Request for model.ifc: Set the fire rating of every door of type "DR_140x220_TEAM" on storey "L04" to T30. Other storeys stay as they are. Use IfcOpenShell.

First a look at what the model holds.

```python
import ifcopenshell
import ifcopenshell.util.element

model = ifcopenshell.open("model.ifc")
print(model.schema)
storey = next(s for s in model.by_type("IfcBuildingStorey") if s.Name == "L04")
doors = [e for e in ifcopenshell.util.element.get_decomposition(storey) if e.is_a("IfcDoor")]
seen = {}
for e in doors:
    element_type = ifcopenshell.util.element.get_type(e)
    key = (element_type.Name if element_type != e and element_type else None, ifcopenshell.util.element.get_pset(e, "Pset_DoorCommon", "FireRating"))
    seen[key] = seen.get(key, 0) + 1
for (name, value), count in sorted(seen.items(), key=str):
    print(count, "x", name, "|", value)
```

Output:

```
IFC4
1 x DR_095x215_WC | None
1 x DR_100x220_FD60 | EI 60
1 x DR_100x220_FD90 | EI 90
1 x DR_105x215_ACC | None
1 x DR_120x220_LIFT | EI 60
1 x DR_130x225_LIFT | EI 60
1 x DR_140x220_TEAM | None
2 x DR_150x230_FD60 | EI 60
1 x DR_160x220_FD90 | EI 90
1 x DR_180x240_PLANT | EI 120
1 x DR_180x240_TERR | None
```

```python
import ifcopenshell
import ifcopenshell.api.pset
import ifcopenshell.util.element

model = ifcopenshell.open("model.ifc")

storey = next(s for s in model.by_type("IfcBuildingStorey") if s.Name == "L04")
doors = [e for e in ifcopenshell.util.element.get_decomposition(storey) if e.is_a("IfcDoor")]

count = 0
for e in doors:
    element_type = ifcopenshell.util.element.get_type(e)
    if element_type in (None, e) or element_type.Name != "DR_140x220_TEAM":
        continue
    # add_pset returns the element's existing set when there is one.
    pset = ifcopenshell.api.pset.add_pset(model, product=e, name="Pset_DoorCommon")
    ifcopenshell.api.pset.edit_pset(model, pset=pset, properties={"FireRating": "T30"})
    count += 1

print(count, "doors updated")

model.write("model_edited.ifc")
```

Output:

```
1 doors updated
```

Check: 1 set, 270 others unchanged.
